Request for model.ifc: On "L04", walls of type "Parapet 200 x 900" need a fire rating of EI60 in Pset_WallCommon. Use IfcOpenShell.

First a look at what the model holds.

```python
import ifcopenshell
import ifcopenshell.util.element

model = ifcopenshell.open("model.ifc")
print(model.schema)
storey = next(s for s in model.by_type("IfcBuildingStorey") if s.Name == "L04")
walls = [e for e in ifcopenshell.util.element.get_decomposition(storey) if e.is_a("IfcWall")]
seen = {}
for e in walls:
    element_type = ifcopenshell.util.element.get_type(e)
    key = (element_type.Name if element_type != e and element_type else None, ifcopenshell.util.element.get_pset(e, "Pset_WallCommon", "FireRating"))
    seen[key] = seen.get(key, 0) + 1
for (name, value), count in sorted(seen.items(), key=str):
    print(count, "x", name, "|", value)
```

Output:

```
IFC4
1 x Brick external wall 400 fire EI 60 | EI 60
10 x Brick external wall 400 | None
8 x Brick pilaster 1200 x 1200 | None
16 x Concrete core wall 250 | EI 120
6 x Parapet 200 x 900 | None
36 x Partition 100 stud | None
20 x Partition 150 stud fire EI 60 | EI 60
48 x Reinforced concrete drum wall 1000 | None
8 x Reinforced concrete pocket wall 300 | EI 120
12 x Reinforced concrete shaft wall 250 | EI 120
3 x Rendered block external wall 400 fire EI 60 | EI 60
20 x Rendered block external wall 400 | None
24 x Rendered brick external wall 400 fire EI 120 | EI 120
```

```python
import ifcopenshell
import ifcopenshell.api.pset
import ifcopenshell.util.element

model = ifcopenshell.open("model.ifc")

storey = next(s for s in model.by_type("IfcBuildingStorey") if s.Name == "L04")
walls = [e for e in ifcopenshell.util.element.get_decomposition(storey) if e.is_a("IfcWall")]

count = 0
for e in walls:
    element_type = ifcopenshell.util.element.get_type(e)
    if element_type in (None, e) or element_type.Name != "Parapet 200 x 900":
        continue
    # add_pset returns the element's existing set when there is one.
    pset = ifcopenshell.api.pset.add_pset(model, product=e, name="Pset_WallCommon")
    ifcopenshell.api.pset.edit_pset(model, pset=pset, properties={"FireRating": "EI60"})
    count += 1

print(count, "walls updated")

model.write("model_v2.ifc")
```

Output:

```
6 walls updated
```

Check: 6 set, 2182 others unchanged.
